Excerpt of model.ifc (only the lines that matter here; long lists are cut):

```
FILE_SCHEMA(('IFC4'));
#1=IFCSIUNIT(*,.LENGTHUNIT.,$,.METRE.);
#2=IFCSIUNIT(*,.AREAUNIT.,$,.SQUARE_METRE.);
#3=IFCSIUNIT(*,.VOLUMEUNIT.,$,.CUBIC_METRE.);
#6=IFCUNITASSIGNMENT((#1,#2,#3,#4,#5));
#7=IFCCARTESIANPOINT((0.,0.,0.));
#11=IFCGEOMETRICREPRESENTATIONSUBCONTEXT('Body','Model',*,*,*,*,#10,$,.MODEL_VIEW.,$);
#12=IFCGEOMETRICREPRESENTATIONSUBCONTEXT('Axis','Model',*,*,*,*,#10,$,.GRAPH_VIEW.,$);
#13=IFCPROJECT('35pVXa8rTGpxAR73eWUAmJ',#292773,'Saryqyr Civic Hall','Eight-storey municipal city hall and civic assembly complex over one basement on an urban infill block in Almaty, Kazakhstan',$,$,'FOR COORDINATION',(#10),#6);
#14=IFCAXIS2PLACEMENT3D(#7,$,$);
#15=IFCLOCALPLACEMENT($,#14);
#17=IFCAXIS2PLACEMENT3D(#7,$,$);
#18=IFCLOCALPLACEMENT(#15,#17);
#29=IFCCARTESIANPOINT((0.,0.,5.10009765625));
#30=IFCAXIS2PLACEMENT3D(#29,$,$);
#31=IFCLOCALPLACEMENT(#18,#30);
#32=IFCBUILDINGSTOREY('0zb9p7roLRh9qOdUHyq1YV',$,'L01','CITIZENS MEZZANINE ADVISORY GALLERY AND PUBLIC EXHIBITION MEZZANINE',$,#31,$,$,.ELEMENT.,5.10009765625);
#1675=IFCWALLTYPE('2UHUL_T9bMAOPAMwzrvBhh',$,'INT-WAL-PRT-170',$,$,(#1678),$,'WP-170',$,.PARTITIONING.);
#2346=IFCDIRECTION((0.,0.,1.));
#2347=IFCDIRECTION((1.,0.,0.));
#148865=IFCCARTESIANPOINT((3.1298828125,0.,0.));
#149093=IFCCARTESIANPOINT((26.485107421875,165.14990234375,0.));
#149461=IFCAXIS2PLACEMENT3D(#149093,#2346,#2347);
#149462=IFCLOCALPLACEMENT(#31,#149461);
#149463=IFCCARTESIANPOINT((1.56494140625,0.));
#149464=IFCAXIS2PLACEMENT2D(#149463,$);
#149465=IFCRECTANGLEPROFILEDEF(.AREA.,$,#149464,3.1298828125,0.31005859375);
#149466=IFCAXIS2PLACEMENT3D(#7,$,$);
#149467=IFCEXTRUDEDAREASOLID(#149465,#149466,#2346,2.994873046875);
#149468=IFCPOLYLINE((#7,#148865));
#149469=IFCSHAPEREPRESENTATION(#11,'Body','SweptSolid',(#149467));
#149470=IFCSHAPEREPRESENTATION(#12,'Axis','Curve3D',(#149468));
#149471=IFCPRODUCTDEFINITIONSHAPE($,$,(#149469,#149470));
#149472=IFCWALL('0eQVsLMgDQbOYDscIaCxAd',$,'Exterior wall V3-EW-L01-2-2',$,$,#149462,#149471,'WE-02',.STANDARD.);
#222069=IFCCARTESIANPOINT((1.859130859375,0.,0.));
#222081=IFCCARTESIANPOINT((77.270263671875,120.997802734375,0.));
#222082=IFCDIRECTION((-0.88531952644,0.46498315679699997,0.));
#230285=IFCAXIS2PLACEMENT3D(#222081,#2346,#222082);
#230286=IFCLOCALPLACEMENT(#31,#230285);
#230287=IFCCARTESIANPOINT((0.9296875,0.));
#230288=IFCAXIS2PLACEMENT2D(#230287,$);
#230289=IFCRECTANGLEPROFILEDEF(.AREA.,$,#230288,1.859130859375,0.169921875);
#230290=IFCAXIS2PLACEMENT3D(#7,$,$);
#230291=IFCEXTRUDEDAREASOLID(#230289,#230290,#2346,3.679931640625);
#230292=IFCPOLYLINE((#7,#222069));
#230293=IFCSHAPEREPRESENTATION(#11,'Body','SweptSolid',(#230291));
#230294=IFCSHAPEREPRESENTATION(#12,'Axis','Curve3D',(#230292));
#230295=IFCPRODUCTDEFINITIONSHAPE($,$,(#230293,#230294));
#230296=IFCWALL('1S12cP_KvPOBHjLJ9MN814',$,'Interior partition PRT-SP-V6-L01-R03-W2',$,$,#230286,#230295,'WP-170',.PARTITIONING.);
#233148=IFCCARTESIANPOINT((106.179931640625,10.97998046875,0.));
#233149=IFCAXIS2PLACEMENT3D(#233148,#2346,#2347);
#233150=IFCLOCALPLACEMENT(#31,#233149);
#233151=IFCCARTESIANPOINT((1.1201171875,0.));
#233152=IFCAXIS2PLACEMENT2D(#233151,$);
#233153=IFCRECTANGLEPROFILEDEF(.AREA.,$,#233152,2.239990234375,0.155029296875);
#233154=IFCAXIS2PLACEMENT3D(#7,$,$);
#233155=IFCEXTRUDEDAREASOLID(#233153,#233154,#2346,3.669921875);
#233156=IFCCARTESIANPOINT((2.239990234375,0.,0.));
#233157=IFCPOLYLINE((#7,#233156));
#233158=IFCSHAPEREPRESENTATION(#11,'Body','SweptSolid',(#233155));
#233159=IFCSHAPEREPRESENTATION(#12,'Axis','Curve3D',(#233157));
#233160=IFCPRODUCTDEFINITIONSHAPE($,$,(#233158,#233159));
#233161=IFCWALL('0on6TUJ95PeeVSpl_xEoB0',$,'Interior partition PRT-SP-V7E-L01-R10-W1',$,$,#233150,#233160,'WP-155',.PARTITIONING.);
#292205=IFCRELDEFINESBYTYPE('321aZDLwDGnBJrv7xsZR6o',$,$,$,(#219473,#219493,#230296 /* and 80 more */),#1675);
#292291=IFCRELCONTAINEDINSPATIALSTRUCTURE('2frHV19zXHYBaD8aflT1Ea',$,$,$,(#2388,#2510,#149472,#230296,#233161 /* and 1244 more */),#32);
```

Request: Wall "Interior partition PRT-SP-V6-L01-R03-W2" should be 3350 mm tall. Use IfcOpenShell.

```python
import ifcopenshell
import ifcopenshell.geom
import ifcopenshell.util.representation
import ifcopenshell.util.shape

model = ifcopenshell.open("model.ifc")
settings = ifcopenshell.geom.settings()


def volume(element):
    """Net volume in cubic metres, openings subtracted."""
    shape = ifcopenshell.geom.create_shape(settings, element)
    return ifcopenshell.util.shape.get_volume(shape.geometry)


wall = model.by_id(230296)
before = volume(wall)

body = ifcopenshell.util.representation.get_representation(wall, "Model", "Body")
solid = body.Items[0]
old_height = solid.Depth
solid.Depth = 3.35
after = volume(wall)

print(f"height {old_height:g} -> {solid.Depth:g}, volume {before:.3f} -> {after:.3f} m3")

model.write("model_edited.ifc")
```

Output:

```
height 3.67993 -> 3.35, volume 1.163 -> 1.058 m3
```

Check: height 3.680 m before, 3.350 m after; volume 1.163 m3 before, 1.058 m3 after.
